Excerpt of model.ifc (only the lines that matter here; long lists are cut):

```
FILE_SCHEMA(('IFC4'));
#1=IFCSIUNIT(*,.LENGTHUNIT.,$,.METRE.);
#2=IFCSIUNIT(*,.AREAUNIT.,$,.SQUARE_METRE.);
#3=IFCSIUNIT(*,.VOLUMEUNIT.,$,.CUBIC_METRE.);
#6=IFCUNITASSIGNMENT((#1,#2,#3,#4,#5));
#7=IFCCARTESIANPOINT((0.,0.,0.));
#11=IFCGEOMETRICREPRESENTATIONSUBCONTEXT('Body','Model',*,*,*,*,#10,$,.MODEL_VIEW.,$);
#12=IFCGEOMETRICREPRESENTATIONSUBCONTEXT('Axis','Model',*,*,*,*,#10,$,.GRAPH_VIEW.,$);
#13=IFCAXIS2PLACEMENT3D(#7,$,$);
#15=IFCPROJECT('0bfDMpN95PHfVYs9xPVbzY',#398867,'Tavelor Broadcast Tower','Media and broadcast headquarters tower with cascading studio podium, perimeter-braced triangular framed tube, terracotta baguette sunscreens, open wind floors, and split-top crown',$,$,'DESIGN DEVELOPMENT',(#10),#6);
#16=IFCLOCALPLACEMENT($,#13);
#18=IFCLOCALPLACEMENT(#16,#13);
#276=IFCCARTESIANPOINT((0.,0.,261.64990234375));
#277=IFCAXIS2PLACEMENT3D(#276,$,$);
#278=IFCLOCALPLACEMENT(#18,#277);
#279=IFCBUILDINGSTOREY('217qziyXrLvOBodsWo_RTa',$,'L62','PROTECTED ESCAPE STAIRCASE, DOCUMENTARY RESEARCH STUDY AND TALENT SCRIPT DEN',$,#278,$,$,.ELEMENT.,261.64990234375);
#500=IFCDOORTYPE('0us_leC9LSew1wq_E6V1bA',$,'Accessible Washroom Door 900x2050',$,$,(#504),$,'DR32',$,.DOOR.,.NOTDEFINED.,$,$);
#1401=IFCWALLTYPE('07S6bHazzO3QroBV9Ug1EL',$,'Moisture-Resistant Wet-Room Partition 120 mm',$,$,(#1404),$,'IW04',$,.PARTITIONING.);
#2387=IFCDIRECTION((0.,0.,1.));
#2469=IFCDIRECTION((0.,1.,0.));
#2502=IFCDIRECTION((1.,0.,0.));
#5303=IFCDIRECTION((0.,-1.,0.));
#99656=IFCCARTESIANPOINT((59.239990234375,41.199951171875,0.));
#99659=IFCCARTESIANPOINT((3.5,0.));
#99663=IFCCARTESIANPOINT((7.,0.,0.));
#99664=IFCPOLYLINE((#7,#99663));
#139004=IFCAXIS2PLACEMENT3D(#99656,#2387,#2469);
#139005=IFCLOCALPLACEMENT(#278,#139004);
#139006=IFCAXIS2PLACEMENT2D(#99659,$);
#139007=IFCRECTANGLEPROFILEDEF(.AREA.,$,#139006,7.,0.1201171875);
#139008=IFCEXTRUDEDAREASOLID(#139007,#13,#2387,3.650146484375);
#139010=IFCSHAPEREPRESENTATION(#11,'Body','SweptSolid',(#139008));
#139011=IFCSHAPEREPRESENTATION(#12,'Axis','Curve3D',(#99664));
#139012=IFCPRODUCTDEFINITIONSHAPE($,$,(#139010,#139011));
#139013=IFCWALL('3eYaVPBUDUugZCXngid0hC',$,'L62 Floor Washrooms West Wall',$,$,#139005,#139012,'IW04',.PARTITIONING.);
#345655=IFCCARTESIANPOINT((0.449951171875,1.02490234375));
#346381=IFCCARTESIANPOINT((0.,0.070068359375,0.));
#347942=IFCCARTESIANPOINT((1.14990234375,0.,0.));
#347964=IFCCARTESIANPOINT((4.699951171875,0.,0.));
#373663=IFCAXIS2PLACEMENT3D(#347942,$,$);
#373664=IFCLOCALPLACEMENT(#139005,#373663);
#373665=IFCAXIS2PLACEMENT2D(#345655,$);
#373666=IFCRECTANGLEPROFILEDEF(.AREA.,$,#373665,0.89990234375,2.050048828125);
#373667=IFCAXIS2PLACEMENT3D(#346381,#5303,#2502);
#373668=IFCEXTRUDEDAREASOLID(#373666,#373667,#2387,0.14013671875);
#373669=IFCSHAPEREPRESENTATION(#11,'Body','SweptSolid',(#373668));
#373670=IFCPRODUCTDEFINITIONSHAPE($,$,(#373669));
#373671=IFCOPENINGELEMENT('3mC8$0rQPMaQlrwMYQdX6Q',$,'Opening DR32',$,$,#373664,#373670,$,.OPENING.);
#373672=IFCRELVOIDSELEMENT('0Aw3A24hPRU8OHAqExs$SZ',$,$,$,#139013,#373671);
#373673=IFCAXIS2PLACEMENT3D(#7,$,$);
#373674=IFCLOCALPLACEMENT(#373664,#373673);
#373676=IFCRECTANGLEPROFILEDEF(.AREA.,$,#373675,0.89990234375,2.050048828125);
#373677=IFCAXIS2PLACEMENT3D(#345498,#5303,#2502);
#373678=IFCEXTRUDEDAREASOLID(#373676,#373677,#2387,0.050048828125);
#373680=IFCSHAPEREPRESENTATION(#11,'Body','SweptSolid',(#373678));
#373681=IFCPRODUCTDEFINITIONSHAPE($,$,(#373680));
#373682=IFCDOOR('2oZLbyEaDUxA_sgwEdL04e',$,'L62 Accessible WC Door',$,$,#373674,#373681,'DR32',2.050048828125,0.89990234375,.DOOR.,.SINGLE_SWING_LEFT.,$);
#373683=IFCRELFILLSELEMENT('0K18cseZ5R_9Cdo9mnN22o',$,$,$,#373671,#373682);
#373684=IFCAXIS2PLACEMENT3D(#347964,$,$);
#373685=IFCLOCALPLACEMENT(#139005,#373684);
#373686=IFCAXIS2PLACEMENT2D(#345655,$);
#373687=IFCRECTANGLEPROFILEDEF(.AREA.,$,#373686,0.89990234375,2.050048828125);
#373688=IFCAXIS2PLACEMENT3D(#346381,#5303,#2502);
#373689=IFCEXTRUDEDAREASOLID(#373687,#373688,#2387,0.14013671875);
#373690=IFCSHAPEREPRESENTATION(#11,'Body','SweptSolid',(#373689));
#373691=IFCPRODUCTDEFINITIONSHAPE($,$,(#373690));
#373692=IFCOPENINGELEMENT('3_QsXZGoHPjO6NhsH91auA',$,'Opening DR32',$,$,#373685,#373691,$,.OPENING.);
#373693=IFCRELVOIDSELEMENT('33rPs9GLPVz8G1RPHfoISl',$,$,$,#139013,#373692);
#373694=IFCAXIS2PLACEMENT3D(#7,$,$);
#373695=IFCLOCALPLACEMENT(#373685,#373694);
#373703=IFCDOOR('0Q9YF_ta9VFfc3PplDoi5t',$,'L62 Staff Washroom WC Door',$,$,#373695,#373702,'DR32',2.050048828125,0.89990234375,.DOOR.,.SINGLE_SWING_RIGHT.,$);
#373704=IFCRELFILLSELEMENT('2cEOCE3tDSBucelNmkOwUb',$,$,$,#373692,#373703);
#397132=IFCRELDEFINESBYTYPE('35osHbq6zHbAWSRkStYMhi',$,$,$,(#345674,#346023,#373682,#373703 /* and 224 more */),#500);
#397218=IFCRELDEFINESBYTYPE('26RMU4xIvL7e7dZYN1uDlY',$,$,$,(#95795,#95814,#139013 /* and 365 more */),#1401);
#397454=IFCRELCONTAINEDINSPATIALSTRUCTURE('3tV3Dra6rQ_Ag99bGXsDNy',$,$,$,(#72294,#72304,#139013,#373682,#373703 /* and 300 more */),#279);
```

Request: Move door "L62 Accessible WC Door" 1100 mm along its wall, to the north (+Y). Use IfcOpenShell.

```python
import ifcopenshell
import ifcopenshell.api.geometry
import ifcopenshell.util.placement
import ifcopenshell.util.unit

model = ifcopenshell.open("model.ifc")
unit_scale = ifcopenshell.util.unit.calculate_unit_scale(model)

door = model.by_guid("2oZLbyEaDUxA_sgwEdL04e")
opening = door.FillsVoids[0].RelatingOpeningElement
wall = opening.VoidsElements[0].RelatingBuildingElement

wall_matrix = ifcopenshell.util.placement.get_local_placement(wall.ObjectPlacement)
shift = wall_matrix[:3, 0] * 1.1 / unit_scale
before = ifcopenshell.util.placement.get_local_placement(door.ObjectPlacement)[:3, 3].copy()

# The door is placed relative to its opening, so it follows when the opening moves.
matrix = ifcopenshell.util.placement.get_local_placement(opening.ObjectPlacement)
matrix[:3, 3] += shift
ifcopenshell.api.geometry.edit_object_placement(
    model, product=opening, matrix=matrix, is_si=False, should_transform_children=True
)

after = ifcopenshell.util.placement.get_local_placement(door.ObjectPlacement)[:3, 3]
print("door moved by", (after - before).round(3) + 0.0)

model.write("model_updated.ifc")
```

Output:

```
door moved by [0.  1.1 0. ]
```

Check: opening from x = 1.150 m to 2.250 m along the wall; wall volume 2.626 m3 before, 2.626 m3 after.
